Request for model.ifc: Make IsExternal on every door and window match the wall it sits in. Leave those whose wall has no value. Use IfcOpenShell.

First a look at what the model holds.

```python
import ifcopenshell
import ifcopenshell.util.element

model = ifcopenshell.open("model.ifc")
print(model.schema)
seen = {}
for e in model.by_type("IfcDoor") + model.by_type("IfcWindow"):
    if not e.FillsVoids:
        continue
    host = e.FillsVoids[0].RelatingOpeningElement.VoidsElements[0].RelatingBuildingElement
    own = ifcopenshell.util.element.get_pset(e, f"Pset_{e.is_a()[3:].removesuffix('StandardCase')}Common", "IsExternal")
    wall = ifcopenshell.util.element.get_pset(host, "Pset_WallCommon", "IsExternal")
    seen[e.is_a(), own, wall] = seen.get((e.is_a(), own, wall), 0) + 1
for (cls, own, wall), count in sorted(seen.items(), key=str):
    print(count, cls, "IsExternal:", own, "| host wall:", wall)
```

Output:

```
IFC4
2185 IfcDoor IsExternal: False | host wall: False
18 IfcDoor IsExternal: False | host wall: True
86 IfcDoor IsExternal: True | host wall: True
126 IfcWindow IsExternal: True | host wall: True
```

```python
import ifcopenshell
import ifcopenshell.api.pset
import ifcopenshell.util.element

model = ifcopenshell.open("model.ifc")

count = 0
for ifc_class, pset_name in (("IfcDoor", "Pset_DoorCommon"), ("IfcWindow", "Pset_WindowCommon")):
    for e in model.by_type(ifc_class):
        if not e.FillsVoids:
            continue
        host = e.FillsVoids[0].RelatingOpeningElement.VoidsElements[0].RelatingBuildingElement
        external = ifcopenshell.util.element.get_pset(host, "Pset_WallCommon", "IsExternal")
        if external is None or ifcopenshell.util.element.get_pset(e, pset_name, "IsExternal") == external:
            continue
        found = ifcopenshell.util.element.get_pset(e, pset_name, should_inherit=False)
        if found:
            pset = model.by_id(found["id"])
            if len(ifcopenshell.util.element.get_elements_by_pset(pset)) > 1:
                pset = ifcopenshell.api.pset.unshare_pset(model, products=[e], pset=pset)[0]
        else:
            pset = ifcopenshell.api.pset.add_pset(model, product=e, name=pset_name)
        ifcopenshell.api.pset.edit_pset(model, pset=pset, properties={"IsExternal": external})
        count += 1

print(count, "updated")

model.write("model_updated.ifc")
```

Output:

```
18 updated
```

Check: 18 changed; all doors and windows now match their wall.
